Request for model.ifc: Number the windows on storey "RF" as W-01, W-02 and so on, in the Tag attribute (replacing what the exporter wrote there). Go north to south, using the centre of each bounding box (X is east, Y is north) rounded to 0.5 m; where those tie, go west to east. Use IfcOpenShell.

First a look at what the model holds.

```python
import ifcopenshell
import ifcopenshell.util.element
import ifcopenshell.util.placement

model = ifcopenshell.open("model.ifc")
print(model.schema)
storey = next(s for s in model.by_type("IfcBuildingStorey") if s.Name == "RF")
windows = [e for e in ifcopenshell.util.element.get_decomposition(storey) if e.is_a("IfcWindow")]
for e in sorted(windows, key=lambda e: e.id()):
    origin = ifcopenshell.util.placement.get_local_placement(e.ObjectPlacement)[:3, 3]
    print(e.id(), e.Tag, e.Name, origin.round(2) + 0.0, sep=" | ")
```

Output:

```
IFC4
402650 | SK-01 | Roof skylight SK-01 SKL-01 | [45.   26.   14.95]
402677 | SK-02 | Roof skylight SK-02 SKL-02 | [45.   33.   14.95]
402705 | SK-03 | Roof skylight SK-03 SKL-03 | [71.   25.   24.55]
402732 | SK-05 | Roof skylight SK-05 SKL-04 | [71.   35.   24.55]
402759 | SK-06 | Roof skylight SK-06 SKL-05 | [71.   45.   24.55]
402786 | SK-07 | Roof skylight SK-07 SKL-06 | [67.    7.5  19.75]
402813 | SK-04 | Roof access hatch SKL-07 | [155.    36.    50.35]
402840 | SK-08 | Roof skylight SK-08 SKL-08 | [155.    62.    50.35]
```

```python
import ifcopenshell
import ifcopenshell.geom
import ifcopenshell.util.element
import ifcopenshell.util.shape

model = ifcopenshell.open("model.ifc")
settings = ifcopenshell.geom.settings()
settings.set("use-world-coords", True)


def centre(element):
    shape = ifcopenshell.geom.create_shape(settings, element)
    return ifcopenshell.util.shape.get_bbox_centroid(shape.geometry)


storey = next(s for s in model.by_type("IfcBuildingStorey") if s.Name == "RF")
windows = [e for e in ifcopenshell.util.element.get_decomposition(storey) if e.is_a("IfcWindow")]

# Insertion points can sit at a corner or the storey origin, so sort by the geometry (in metres).
centres = {e: centre(e) for e in windows}
windows.sort(key=lambda e: (-round(centres[e][1] / 0.5), centres[e][0]))

for i, e in enumerate(windows, start=1):
    number = f"W-{i:02d}"
    e.Tag = number
    print(e.id(), number)

model.write("model_rev.ifc")
```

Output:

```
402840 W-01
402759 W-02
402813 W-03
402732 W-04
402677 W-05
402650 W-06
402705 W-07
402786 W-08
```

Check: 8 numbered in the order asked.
